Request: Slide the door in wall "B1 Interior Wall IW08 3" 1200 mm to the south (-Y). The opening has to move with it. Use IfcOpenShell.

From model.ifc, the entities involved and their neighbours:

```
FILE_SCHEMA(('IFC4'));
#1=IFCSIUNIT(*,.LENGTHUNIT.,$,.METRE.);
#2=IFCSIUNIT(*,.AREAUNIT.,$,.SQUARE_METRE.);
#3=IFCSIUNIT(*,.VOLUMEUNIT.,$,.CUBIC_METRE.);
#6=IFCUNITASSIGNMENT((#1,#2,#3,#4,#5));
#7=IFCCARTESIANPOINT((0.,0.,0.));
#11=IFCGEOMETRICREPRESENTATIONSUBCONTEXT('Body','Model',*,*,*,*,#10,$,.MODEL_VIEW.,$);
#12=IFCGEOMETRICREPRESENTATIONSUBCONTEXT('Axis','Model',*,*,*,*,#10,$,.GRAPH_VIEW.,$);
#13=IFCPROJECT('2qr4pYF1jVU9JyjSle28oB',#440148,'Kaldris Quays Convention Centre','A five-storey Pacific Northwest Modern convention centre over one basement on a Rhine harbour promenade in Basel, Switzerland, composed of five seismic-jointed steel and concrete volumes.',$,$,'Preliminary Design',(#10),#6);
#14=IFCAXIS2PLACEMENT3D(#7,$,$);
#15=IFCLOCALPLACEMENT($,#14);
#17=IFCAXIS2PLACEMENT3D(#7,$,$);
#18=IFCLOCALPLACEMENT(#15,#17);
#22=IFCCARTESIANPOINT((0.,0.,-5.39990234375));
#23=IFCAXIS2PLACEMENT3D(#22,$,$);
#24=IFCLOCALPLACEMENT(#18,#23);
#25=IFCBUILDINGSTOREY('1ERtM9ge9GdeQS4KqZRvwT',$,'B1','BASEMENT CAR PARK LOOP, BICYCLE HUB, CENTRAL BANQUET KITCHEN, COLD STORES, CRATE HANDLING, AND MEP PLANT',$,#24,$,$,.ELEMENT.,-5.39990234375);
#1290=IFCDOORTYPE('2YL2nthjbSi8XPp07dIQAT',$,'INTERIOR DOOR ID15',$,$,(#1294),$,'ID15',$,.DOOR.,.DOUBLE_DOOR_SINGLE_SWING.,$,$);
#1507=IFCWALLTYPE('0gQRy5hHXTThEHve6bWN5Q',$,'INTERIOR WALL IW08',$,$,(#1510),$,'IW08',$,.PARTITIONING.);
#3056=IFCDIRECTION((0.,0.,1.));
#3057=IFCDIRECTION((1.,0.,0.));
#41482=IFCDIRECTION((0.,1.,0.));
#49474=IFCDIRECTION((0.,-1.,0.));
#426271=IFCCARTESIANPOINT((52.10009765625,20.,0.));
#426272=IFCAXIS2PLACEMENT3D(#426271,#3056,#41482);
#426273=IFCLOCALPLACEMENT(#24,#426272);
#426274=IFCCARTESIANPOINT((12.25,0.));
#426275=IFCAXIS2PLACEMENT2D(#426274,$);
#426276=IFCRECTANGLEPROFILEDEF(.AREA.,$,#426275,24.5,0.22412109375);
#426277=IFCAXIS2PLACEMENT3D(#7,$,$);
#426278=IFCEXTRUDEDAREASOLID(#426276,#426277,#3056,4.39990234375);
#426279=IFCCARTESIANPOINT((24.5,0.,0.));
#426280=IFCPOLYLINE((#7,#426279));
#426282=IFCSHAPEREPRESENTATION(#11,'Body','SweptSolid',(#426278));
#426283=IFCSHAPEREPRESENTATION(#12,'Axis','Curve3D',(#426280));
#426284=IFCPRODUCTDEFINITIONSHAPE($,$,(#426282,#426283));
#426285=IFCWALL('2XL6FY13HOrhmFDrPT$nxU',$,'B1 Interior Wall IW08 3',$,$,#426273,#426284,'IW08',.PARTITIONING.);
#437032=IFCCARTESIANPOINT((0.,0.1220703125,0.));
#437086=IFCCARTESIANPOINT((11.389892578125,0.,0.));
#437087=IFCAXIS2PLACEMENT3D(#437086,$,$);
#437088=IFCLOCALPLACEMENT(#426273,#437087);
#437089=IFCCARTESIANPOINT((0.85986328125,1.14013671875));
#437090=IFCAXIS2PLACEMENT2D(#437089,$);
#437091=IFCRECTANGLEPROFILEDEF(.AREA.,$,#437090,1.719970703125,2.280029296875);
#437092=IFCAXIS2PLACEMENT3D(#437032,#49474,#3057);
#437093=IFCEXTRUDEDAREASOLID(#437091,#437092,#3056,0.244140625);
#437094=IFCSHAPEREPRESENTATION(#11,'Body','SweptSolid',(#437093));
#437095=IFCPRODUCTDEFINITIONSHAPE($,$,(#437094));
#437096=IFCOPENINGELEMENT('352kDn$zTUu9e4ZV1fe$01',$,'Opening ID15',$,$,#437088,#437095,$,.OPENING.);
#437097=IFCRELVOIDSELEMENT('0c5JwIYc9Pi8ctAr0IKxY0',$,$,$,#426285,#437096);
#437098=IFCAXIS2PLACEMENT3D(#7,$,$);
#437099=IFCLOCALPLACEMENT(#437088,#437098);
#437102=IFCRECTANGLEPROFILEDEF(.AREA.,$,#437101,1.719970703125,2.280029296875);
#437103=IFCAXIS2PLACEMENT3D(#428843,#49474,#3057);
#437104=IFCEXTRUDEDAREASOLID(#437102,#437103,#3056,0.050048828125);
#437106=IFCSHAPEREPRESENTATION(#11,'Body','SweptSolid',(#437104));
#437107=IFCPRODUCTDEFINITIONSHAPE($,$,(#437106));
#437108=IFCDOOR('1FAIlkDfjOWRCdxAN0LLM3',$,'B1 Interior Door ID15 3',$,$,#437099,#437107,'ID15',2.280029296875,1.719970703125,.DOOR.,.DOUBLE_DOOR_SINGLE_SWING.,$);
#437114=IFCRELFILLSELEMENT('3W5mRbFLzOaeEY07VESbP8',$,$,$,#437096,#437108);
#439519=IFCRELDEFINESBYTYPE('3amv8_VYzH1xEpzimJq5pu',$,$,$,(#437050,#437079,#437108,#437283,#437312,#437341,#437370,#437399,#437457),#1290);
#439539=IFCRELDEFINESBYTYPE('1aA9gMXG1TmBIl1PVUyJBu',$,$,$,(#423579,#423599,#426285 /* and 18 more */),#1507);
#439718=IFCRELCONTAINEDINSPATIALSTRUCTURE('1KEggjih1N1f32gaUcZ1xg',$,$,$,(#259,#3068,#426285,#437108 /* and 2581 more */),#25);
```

```python
import ifcopenshell
import ifcopenshell.api.geometry
import ifcopenshell.util.placement
import ifcopenshell.util.unit

model = ifcopenshell.open("model.ifc")
unit_scale = ifcopenshell.util.unit.calculate_unit_scale(model)

door = model.by_guid("1FAIlkDfjOWRCdxAN0LLM3")
opening = door.FillsVoids[0].RelatingOpeningElement
wall = opening.VoidsElements[0].RelatingBuildingElement

wall_matrix = ifcopenshell.util.placement.get_local_placement(wall.ObjectPlacement)
shift = wall_matrix[:3, 0] * -1.2 / unit_scale
before = ifcopenshell.util.placement.get_local_placement(door.ObjectPlacement)[:3, 3].copy()

# The door is placed relative to its opening, so it follows when the opening moves.
matrix = ifcopenshell.util.placement.get_local_placement(opening.ObjectPlacement)
matrix[:3, 3] += shift
ifcopenshell.api.geometry.edit_object_placement(
    model, product=opening, matrix=matrix, is_si=False, should_transform_children=True
)

after = ifcopenshell.util.placement.get_local_placement(door.ObjectPlacement)[:3, 3]
print("door moved by", (after - before).round(3) + 0.0)

model.write("model_rev.ifc")
```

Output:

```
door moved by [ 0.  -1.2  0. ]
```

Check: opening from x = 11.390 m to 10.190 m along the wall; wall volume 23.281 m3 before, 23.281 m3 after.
